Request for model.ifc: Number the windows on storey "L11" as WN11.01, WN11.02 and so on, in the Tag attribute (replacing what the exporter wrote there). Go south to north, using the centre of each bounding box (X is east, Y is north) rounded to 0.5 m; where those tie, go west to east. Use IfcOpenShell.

First a look at what the model holds.

```python
import ifcopenshell
import ifcopenshell.util.element
import ifcopenshell.util.placement

model = ifcopenshell.open("model.ifc")
print(model.schema)
storey = next(s for s in model.by_type("IfcBuildingStorey") if s.Name == "L11")
windows = [e for e in ifcopenshell.util.element.get_decomposition(storey) if e.is_a("IfcWindow")]
for e in sorted(windows, key=lambda e: e.id()):
    origin = ifcopenshell.util.placement.get_local_placement(e.ObjectPlacement)[:3, 3]
    print(e.id(), e.Tag, e.Name, origin.round(2) + 0.0, sep=" | ")
```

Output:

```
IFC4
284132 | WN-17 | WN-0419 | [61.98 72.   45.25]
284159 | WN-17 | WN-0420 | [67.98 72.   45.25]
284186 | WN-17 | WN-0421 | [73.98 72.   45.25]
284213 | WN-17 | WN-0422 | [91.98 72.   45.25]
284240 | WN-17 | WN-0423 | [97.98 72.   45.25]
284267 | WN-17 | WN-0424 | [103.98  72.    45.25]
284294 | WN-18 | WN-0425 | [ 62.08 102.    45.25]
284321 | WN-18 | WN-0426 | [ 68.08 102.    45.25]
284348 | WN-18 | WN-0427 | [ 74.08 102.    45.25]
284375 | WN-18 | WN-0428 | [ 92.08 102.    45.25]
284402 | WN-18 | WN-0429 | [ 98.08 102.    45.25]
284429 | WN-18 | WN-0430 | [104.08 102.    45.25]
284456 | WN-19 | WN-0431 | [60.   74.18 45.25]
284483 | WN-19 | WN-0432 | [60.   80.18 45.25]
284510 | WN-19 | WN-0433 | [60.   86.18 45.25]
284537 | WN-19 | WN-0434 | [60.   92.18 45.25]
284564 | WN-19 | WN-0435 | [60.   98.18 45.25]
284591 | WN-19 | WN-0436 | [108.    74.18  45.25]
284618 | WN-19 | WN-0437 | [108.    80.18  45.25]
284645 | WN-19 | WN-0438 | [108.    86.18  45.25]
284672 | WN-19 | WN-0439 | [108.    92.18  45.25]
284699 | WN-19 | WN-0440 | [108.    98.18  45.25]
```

```python
import ifcopenshell
import ifcopenshell.geom
import ifcopenshell.util.element
import ifcopenshell.util.shape

model = ifcopenshell.open("model.ifc")
settings = ifcopenshell.geom.settings()
settings.set("use-world-coords", True)


def centre(element):
    shape = ifcopenshell.geom.create_shape(settings, element)
    return ifcopenshell.util.shape.get_bbox_centroid(shape.geometry)


storey = next(s for s in model.by_type("IfcBuildingStorey") if s.Name == "L11")
windows = [e for e in ifcopenshell.util.element.get_decomposition(storey) if e.is_a("IfcWindow")]

# Insertion points can sit at a corner or the storey origin, so sort by the geometry (in metres).
centres = {e: centre(e) for e in windows}
windows.sort(key=lambda e: (round(centres[e][1] / 0.5), centres[e][0]))

for i, e in enumerate(windows, start=1):
    number = f"WN11.{i:02d}"
    e.Tag = number
    print(e.id(), number)

model.write("model_edited.ifc")
```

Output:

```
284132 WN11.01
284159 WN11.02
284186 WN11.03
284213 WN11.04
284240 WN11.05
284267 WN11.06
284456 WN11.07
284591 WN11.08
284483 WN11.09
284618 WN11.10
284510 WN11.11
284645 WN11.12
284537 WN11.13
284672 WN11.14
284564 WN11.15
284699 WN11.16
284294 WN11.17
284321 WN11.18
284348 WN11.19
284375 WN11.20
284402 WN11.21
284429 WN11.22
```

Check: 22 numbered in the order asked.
